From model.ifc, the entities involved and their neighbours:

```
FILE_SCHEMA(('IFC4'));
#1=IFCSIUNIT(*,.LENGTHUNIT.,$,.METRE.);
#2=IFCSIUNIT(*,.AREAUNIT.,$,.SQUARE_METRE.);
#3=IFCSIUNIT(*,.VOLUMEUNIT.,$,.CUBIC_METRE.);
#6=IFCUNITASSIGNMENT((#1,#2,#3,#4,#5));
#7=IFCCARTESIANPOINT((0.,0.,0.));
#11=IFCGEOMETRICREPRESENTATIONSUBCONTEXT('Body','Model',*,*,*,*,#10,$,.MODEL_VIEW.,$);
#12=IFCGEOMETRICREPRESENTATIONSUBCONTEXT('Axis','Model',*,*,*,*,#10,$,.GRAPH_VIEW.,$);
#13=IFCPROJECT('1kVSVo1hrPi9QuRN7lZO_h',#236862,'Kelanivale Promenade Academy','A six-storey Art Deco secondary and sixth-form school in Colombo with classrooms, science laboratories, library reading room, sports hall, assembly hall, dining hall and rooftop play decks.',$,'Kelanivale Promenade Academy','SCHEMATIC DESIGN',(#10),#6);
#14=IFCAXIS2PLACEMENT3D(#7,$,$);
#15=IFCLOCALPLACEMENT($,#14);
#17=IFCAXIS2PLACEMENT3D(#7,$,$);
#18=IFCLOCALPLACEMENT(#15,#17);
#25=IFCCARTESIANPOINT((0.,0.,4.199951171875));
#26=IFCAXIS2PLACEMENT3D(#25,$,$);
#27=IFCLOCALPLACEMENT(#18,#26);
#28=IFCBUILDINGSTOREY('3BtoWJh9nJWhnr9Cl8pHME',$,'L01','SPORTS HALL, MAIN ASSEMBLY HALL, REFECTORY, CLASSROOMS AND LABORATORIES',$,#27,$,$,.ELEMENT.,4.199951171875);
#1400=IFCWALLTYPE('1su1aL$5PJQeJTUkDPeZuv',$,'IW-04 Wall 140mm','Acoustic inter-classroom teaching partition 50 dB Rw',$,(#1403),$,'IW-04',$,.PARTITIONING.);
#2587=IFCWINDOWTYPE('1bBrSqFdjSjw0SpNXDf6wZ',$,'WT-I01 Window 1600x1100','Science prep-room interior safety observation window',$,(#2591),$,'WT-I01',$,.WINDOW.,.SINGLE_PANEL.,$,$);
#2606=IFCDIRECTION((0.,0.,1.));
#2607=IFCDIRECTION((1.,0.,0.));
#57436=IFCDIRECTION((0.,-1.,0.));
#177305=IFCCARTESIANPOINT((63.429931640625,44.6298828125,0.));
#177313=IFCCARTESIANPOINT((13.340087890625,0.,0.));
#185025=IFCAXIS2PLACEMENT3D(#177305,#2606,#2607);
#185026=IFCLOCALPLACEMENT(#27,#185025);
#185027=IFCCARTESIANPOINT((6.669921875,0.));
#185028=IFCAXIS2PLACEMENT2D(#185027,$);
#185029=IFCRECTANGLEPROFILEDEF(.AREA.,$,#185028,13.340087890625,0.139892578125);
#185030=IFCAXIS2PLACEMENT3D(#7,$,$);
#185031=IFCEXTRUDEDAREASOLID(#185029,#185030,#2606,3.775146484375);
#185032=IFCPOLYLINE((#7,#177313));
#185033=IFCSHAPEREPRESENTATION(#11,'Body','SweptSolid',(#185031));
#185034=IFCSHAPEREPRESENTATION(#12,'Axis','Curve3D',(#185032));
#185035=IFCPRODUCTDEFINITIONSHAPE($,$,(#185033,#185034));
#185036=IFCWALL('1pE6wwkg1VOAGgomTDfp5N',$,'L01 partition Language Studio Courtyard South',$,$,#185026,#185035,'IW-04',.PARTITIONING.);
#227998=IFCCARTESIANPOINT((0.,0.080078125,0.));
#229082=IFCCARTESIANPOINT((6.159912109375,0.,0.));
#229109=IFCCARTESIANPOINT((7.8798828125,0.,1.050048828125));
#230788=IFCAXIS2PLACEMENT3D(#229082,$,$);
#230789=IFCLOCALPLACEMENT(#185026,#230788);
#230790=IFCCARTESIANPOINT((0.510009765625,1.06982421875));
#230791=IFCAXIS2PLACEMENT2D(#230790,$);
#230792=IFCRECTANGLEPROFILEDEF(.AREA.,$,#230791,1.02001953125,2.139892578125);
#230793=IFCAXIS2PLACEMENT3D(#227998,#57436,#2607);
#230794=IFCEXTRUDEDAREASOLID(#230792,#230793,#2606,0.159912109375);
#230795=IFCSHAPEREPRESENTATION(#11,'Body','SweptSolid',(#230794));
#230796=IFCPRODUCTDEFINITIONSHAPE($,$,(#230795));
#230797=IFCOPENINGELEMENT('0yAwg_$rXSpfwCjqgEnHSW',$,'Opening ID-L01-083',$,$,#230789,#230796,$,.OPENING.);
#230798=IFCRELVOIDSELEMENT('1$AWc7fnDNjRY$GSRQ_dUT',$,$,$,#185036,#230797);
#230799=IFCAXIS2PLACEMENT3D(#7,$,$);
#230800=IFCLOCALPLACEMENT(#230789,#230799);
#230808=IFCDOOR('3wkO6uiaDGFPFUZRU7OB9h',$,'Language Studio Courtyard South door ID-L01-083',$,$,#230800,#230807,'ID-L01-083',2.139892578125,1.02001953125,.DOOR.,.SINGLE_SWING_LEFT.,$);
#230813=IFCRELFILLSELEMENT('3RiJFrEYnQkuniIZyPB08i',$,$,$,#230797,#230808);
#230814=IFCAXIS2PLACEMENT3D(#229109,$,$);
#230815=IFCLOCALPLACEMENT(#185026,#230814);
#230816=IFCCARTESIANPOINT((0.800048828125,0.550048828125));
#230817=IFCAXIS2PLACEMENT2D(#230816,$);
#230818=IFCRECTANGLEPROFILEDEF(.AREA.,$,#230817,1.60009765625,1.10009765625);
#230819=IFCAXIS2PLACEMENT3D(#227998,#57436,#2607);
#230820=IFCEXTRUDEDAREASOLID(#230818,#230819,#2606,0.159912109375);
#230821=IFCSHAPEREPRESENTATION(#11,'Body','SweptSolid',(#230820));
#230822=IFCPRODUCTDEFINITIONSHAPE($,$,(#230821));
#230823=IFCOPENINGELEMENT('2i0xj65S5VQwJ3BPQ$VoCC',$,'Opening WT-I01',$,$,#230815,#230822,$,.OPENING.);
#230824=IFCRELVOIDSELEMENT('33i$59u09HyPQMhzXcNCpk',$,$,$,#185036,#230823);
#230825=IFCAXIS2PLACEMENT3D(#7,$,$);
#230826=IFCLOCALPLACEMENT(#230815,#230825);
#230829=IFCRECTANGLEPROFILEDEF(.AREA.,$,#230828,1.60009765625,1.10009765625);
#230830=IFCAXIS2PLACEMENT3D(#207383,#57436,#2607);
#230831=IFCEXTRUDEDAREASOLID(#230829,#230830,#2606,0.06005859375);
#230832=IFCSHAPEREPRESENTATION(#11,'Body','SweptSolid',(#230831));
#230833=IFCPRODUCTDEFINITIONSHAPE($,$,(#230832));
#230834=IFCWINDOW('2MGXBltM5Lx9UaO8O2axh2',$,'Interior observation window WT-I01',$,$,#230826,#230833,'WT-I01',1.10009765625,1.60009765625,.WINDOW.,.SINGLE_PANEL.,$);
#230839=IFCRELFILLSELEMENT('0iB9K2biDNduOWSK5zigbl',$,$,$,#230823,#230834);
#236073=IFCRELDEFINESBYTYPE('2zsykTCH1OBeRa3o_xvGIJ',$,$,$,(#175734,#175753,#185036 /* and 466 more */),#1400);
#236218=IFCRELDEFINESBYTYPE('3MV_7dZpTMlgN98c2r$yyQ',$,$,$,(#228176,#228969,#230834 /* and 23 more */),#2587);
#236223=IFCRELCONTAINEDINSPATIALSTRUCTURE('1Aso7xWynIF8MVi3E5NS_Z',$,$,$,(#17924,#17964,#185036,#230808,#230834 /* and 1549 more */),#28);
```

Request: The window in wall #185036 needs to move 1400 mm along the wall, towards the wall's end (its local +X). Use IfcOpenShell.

```python
import ifcopenshell
import ifcopenshell.api.geometry
import ifcopenshell.util.placement

model = ifcopenshell.open("model.ifc")

window = model.by_guid("2MGXBltM5Lx9UaO8O2axh2")
opening = window.FillsVoids[0].RelatingOpeningElement
wall = opening.VoidsElements[0].RelatingBuildingElement

wall_matrix = ifcopenshell.util.placement.get_local_placement(wall.ObjectPlacement)
shift = wall_matrix[:3, 0] * 1.4
before = ifcopenshell.util.placement.get_local_placement(window.ObjectPlacement)[:3, 3].copy()

# The window is placed relative to its opening, so it follows when the opening moves.
matrix = ifcopenshell.util.placement.get_local_placement(opening.ObjectPlacement)
matrix[:3, 3] += shift
ifcopenshell.api.geometry.edit_object_placement(
    model, product=opening, matrix=matrix, is_si=False, should_transform_children=True
)

after = ifcopenshell.util.placement.get_local_placement(window.ObjectPlacement)[:3, 3]
print("window moved by", (after - before).round(3) + 0.0)

model.write("model_v2.ifc")
```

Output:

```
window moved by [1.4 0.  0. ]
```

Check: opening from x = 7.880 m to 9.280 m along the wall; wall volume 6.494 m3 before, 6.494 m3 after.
